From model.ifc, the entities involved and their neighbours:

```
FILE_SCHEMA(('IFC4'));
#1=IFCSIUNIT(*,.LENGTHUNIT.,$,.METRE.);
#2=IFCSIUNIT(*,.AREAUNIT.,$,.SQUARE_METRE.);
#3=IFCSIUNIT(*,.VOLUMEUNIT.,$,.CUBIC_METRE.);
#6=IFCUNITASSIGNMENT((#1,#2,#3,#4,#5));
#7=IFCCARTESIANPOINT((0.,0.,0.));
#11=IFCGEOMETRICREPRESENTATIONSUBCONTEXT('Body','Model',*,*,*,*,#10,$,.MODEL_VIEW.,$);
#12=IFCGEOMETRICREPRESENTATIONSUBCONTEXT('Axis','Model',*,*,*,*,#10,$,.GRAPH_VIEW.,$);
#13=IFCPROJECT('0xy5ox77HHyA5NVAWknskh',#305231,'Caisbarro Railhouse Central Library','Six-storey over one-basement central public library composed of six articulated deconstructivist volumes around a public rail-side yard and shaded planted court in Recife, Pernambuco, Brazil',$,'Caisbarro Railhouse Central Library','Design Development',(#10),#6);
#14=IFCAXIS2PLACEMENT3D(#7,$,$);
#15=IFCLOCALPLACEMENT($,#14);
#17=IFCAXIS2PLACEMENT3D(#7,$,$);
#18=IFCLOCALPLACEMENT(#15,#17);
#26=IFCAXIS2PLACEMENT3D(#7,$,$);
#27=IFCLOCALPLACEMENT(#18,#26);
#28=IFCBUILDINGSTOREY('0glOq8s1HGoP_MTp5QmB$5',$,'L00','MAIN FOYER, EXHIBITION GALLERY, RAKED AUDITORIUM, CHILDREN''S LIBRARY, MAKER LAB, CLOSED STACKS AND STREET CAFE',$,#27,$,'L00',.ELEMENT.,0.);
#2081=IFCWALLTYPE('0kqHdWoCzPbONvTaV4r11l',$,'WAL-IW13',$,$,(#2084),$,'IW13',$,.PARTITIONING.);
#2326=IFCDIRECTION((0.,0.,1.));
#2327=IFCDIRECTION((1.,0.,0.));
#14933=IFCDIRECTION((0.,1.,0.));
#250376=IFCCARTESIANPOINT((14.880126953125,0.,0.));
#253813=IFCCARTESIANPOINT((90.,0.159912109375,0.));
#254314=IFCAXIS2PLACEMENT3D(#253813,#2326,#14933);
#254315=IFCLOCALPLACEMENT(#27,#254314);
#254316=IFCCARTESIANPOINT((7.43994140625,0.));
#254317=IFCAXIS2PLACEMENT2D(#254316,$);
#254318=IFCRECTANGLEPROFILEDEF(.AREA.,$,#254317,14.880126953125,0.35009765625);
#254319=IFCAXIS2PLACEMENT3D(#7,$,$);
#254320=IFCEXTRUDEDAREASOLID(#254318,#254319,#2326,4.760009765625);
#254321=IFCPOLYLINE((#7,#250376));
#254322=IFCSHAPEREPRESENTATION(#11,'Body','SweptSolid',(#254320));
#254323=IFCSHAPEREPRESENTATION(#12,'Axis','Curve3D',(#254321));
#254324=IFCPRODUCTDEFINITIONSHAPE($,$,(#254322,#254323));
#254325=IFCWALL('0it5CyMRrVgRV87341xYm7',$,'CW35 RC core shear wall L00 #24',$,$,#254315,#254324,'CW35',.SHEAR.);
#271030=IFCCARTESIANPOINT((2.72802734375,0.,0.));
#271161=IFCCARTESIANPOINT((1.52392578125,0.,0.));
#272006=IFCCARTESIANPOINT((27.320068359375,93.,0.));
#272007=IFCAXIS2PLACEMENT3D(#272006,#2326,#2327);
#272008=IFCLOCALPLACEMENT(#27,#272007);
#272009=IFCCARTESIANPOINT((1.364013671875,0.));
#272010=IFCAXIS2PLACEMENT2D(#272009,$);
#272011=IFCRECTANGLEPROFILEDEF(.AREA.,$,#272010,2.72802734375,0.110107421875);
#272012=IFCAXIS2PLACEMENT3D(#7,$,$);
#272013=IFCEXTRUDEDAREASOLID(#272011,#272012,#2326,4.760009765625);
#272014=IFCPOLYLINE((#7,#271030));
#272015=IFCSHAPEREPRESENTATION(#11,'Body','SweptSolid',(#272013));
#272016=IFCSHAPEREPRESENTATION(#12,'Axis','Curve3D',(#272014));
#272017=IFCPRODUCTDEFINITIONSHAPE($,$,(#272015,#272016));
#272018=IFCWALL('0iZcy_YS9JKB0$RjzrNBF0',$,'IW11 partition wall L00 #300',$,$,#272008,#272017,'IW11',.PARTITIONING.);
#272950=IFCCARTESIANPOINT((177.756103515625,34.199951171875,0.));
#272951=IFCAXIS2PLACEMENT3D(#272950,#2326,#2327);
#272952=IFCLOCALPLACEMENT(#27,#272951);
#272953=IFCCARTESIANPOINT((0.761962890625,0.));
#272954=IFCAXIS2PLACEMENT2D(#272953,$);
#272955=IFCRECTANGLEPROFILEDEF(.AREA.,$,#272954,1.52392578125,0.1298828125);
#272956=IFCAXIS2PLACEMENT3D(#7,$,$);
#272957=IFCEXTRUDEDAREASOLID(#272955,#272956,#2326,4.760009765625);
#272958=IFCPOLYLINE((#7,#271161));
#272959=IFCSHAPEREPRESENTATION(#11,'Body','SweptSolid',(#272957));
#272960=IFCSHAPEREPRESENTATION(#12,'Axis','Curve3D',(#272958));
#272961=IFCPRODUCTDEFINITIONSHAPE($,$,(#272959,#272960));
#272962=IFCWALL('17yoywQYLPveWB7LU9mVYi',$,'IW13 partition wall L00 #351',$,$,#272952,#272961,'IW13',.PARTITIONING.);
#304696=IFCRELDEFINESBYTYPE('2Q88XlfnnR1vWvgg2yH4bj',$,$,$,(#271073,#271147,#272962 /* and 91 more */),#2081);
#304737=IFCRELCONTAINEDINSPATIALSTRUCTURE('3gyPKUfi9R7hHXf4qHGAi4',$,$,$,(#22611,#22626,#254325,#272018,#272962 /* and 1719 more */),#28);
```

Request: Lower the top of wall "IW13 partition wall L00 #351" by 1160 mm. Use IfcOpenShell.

```python
import ifcopenshell
import ifcopenshell.geom
import ifcopenshell.util.representation
import ifcopenshell.util.shape

model = ifcopenshell.open("model.ifc")
settings = ifcopenshell.geom.settings()


def volume(element):
    """Net volume in cubic metres, openings subtracted."""
    shape = ifcopenshell.geom.create_shape(settings, element)
    return ifcopenshell.util.shape.get_volume(shape.geometry)


wall = model.by_guid("17yoywQYLPveWB7LU9mVYi")
before = volume(wall)

body = ifcopenshell.util.representation.get_representation(wall, "Model", "Body")
solid = body.Items[0]
old_height = solid.Depth
solid.Depth -= 1.16
after = volume(wall)

print(f"height {old_height:g} -> {solid.Depth:g}, volume {before:.3f} -> {after:.3f} m3")

model.write("model_rev.ifc")
```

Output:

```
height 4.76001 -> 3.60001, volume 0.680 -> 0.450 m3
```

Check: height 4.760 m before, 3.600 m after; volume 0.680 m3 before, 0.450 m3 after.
